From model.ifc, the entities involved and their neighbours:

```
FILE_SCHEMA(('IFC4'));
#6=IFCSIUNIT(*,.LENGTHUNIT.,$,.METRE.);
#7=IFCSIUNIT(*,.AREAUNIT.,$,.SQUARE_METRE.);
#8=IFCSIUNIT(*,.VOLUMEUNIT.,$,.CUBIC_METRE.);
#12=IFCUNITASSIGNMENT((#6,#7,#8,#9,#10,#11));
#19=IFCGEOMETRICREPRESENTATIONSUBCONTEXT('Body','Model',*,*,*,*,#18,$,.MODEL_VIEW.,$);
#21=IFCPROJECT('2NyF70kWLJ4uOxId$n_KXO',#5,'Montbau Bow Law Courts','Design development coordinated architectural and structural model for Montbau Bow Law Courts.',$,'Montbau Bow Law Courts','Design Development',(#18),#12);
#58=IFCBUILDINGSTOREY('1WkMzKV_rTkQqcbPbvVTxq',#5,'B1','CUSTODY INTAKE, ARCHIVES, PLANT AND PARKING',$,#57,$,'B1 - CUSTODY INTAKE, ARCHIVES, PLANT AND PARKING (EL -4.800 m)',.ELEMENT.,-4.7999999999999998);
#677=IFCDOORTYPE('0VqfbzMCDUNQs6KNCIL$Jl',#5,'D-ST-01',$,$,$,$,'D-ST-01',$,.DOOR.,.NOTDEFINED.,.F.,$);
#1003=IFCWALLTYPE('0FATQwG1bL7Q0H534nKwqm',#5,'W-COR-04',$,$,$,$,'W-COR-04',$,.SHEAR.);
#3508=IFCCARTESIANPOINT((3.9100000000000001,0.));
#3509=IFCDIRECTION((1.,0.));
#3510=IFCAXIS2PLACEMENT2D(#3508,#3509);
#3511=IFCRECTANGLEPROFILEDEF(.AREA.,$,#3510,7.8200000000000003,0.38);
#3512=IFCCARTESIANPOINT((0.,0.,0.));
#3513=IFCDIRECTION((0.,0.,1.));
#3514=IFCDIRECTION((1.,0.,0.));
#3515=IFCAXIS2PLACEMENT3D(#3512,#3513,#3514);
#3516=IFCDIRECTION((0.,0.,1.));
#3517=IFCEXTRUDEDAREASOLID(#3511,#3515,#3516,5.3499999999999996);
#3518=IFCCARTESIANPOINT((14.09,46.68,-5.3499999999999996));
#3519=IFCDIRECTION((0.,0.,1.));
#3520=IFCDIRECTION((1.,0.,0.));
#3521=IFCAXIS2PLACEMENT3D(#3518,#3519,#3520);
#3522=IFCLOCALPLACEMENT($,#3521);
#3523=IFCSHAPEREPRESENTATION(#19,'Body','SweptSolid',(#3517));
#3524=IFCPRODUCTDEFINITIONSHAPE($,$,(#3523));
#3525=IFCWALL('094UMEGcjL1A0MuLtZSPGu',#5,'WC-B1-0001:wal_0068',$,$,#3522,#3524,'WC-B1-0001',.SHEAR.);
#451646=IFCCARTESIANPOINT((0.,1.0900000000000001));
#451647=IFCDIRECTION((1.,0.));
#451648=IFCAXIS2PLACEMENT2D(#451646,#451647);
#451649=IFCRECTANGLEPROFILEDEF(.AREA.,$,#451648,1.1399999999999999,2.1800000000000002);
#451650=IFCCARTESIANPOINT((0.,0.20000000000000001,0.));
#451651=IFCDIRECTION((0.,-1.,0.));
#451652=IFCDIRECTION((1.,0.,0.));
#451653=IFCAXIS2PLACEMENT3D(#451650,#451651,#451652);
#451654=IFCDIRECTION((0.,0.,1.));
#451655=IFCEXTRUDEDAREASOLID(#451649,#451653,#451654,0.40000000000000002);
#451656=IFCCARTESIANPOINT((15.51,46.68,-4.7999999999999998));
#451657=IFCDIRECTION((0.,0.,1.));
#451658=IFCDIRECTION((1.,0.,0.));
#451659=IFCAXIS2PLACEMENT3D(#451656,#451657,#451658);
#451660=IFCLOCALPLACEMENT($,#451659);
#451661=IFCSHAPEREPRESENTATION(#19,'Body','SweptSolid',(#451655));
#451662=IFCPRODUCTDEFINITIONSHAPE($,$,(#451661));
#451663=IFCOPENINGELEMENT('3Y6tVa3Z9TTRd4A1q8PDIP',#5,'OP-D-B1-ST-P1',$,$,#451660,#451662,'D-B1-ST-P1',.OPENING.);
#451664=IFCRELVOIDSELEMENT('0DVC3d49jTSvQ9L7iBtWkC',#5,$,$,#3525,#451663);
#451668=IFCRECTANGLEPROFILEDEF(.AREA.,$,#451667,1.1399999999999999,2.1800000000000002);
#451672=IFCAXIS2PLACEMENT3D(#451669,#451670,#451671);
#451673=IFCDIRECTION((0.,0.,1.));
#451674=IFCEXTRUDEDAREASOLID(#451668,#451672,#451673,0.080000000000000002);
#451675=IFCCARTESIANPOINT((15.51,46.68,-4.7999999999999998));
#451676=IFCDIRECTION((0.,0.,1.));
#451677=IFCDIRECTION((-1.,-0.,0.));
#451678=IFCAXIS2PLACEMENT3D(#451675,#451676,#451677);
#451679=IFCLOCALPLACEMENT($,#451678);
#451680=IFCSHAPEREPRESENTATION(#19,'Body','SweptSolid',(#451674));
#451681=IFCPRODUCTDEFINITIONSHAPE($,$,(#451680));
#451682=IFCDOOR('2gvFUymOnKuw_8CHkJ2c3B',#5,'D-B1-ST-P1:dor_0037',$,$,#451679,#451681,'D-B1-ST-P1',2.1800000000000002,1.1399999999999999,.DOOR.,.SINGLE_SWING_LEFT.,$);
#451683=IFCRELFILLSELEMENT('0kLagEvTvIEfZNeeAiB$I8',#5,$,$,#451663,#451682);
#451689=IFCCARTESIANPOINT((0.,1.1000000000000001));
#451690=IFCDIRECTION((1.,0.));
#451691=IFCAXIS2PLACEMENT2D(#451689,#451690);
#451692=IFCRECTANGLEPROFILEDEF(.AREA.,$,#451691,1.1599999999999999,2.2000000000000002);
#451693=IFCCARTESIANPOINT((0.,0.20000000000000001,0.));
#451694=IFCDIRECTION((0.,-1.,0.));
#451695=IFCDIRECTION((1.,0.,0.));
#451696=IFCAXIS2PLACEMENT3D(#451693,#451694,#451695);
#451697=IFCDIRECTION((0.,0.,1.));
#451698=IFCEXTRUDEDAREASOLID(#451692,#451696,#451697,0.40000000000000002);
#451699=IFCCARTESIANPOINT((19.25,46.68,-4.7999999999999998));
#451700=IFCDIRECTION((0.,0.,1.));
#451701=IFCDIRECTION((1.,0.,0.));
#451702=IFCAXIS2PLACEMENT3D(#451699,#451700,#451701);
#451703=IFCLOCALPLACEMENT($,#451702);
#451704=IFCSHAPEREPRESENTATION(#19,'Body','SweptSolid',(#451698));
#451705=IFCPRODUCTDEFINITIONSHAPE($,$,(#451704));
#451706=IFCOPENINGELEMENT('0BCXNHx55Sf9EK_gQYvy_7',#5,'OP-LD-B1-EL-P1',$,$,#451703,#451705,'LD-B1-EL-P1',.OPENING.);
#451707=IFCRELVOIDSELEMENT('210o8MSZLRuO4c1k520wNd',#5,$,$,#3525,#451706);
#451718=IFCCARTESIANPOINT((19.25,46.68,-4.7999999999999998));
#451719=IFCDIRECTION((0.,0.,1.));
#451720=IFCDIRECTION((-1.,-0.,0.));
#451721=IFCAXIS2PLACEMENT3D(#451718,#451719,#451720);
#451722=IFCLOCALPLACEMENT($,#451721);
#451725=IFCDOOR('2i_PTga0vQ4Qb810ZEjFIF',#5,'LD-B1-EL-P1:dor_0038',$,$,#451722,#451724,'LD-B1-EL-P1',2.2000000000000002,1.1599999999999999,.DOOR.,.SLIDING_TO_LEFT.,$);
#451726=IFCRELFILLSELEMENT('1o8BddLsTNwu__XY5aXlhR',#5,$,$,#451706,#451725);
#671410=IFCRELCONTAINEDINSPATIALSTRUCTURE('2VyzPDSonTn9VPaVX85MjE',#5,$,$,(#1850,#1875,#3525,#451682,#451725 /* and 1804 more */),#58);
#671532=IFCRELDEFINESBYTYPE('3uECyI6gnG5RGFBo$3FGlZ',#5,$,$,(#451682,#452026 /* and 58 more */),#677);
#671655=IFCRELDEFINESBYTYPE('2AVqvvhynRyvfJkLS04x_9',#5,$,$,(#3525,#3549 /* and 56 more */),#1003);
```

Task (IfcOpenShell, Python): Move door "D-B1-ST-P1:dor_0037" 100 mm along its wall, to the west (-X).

```python
import ifcopenshell
import ifcopenshell.api.geometry
import ifcopenshell.util.placement
import ifcopenshell.util.unit

model = ifcopenshell.open("model.ifc")
unit_scale = ifcopenshell.util.unit.calculate_unit_scale(model)

door = model.by_id(451682)
opening = door.FillsVoids[0].RelatingOpeningElement
wall = opening.VoidsElements[0].RelatingBuildingElement

wall_matrix = ifcopenshell.util.placement.get_local_placement(wall.ObjectPlacement)
shift = wall_matrix[:3, 0] * -0.1 / unit_scale
before = ifcopenshell.util.placement.get_local_placement(door.ObjectPlacement)[:3, 3].copy()

# The door is not placed relative to its opening, so move both.
for product in (opening, door):
    matrix = ifcopenshell.util.placement.get_local_placement(product.ObjectPlacement)
    matrix[:3, 3] += shift
    ifcopenshell.api.geometry.edit_object_placement(model, product=product, matrix=matrix, is_si=False)

after = ifcopenshell.util.placement.get_local_placement(door.ObjectPlacement)[:3, 3]
print("door moved by", (after - before).round(3) + 0.0)

model.write("model_v2.ifc")
```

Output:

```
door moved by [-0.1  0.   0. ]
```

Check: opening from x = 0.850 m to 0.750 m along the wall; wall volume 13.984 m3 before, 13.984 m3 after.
